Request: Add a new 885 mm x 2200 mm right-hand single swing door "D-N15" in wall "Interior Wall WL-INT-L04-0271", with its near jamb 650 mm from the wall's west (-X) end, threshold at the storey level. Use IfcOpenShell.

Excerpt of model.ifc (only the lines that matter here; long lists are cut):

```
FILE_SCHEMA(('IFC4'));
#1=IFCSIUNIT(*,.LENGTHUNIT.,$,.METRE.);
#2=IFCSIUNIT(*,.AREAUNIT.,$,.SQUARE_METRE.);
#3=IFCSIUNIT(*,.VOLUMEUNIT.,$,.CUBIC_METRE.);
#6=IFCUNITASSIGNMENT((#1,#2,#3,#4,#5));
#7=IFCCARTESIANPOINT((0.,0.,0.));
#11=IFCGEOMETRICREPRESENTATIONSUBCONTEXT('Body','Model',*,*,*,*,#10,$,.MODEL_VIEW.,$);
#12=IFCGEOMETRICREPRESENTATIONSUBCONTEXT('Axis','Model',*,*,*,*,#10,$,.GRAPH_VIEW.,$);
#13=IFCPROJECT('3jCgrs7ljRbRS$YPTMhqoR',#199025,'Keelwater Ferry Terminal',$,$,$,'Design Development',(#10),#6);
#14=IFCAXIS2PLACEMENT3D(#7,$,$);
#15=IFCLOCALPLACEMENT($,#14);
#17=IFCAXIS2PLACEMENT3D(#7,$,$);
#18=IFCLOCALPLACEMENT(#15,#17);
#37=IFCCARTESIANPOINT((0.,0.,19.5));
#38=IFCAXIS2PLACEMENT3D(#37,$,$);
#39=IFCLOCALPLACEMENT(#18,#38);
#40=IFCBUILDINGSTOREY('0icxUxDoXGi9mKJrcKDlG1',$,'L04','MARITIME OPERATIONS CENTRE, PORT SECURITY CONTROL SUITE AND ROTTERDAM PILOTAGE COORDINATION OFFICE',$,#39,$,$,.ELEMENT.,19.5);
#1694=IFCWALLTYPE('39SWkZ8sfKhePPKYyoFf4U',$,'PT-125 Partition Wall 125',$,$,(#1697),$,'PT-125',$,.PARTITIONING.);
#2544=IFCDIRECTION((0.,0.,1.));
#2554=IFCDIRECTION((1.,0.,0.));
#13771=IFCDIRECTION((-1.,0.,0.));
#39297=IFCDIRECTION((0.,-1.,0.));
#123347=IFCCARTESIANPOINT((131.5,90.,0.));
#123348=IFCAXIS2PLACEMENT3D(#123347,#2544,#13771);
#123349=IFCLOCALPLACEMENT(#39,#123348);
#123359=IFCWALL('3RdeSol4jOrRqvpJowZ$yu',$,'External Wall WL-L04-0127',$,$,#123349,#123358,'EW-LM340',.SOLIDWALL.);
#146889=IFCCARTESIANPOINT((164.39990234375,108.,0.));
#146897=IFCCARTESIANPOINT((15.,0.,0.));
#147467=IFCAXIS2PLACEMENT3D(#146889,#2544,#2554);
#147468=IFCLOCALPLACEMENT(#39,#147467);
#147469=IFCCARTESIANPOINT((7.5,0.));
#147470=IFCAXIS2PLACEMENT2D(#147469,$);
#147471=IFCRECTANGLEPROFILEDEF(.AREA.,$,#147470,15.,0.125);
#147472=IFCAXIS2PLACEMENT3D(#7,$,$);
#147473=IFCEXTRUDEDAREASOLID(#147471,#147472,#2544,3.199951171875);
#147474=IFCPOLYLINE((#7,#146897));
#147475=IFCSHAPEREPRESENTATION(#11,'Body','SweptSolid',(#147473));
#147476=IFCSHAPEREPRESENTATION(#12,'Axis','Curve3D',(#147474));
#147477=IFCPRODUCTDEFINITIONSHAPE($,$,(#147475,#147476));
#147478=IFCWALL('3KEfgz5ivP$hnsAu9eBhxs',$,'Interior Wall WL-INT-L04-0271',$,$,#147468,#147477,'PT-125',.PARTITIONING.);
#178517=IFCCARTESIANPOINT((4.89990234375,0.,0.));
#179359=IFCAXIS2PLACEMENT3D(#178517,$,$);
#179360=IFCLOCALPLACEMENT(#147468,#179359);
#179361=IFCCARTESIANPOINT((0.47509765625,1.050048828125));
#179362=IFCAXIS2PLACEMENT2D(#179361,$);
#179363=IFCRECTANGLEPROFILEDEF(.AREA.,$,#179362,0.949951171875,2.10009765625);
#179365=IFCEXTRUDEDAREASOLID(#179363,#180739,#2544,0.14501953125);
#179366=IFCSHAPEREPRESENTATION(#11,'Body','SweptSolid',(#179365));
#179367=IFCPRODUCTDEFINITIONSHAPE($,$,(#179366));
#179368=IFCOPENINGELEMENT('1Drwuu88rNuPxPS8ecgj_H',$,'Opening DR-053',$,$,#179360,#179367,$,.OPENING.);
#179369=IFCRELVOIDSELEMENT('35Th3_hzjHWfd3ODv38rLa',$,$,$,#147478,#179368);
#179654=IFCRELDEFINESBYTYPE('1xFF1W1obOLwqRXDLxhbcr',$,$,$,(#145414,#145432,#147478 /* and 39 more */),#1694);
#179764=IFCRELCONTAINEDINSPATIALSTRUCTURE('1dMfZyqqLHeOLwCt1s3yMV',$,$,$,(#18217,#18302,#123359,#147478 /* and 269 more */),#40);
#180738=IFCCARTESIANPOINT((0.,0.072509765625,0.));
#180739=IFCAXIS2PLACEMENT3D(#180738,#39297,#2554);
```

```python
import numpy as np
import ifcopenshell
import ifcopenshell.api.feature
import ifcopenshell.api.geometry
import ifcopenshell.api.root
import ifcopenshell.api.spatial
import ifcopenshell.geom
import ifcopenshell.util.element
import ifcopenshell.util.placement
import ifcopenshell.util.representation
import ifcopenshell.util.shape
import ifcopenshell.util.unit

model = ifcopenshell.open("model.ifc")
unit_scale = ifcopenshell.util.unit.calculate_unit_scale(model)
settings = ifcopenshell.geom.settings()


def volume(element):
    """Net volume in cubic metres, openings subtracted."""
    shape = ifcopenshell.geom.create_shape(settings, element)
    return ifcopenshell.util.shape.get_volume(shape.geometry)


wall = model.by_id(147478)
storey = ifcopenshell.util.element.get_container(wall, ifc_class="IfcBuildingStorey")
context = ifcopenshell.util.representation.get_context(model, "Model", "Body", "MODEL_VIEW")
before = volume(wall)

width, height, from_end, sill = 0.885, 2.2, 0.65, 0.0  # metres

# The wall runs along its own X axis, and the end named is its -X end.
wall_shape = ifcopenshell.geom.create_shape(settings, wall)
x, y, z = ifcopenshell.util.shape.get_vertices(wall_shape.geometry).T
start = x.min() + from_end
face, thickness = float(y.min()), float(y.max() - y.min())
wall_matrix = ifcopenshell.util.placement.get_local_placement(wall.ObjectPlacement)
level = ifcopenshell.util.placement.get_local_placement(storey.ObjectPlacement)[2, 3]


def in_wall(x, y):
    """Placement at x, y metres in the wall's axes, at sill height."""
    matrix = wall_matrix.copy()
    matrix[:, 3] = wall_matrix @ np.array([x / unit_scale, y / unit_scale, 0.0, 1.0])
    matrix[2, 3] = level + sill / unit_scale
    return matrix


# Opening: a box that overshoots both wall faces by 50 mm.
opening = ifcopenshell.api.root.create_entity(model, ifc_class="IfcOpeningElement", predefined_type="OPENING")
box = ifcopenshell.api.geometry.add_wall_representation(
    model, context=context, length=width, height=height, thickness=thickness + 0.1
)
ifcopenshell.api.geometry.assign_representation(model, product=opening, representation=box)
ifcopenshell.api.geometry.edit_object_placement(model, product=opening, matrix=in_wall(start, face - 0.05), is_si=False)
ifcopenshell.api.feature.add_feature(model, feature=opening, element=wall)

door = ifcopenshell.api.root.create_entity(model, ifc_class="IfcDoor", name="D-N15", predefined_type="DOOR")
door.OverallWidth, door.OverallHeight = width / unit_scale, height / unit_scale
door.OperationType = "SINGLE_SWING_RIGHT"
body = ifcopenshell.api.geometry.add_door_representation(
    model,
    context=context,
    overall_width=door.OverallWidth,
    overall_height=door.OverallHeight,
    operation_type="SINGLE_SWING_RIGHT",
    lining_properties={"LiningDepth": thickness / unit_scale, "ThresholdDepth": thickness / unit_scale},
)
ifcopenshell.api.geometry.assign_representation(model, product=door, representation=body)
ifcopenshell.api.spatial.assign_container(model, products=[door], relating_structure=storey)
ifcopenshell.api.feature.add_filling(model, opening=opening, element=door)

# The lining spans the wall, so the door starts at the wall face.
ifcopenshell.api.geometry.edit_object_placement(model, product=door, matrix=in_wall(start, face), is_si=False)

after = volume(wall)

print(f"wall volume {before:.3f} -> {after:.3f} m3")

model.write("model-out.ifc")
```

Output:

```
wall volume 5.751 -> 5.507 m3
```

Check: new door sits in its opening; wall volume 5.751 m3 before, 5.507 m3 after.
